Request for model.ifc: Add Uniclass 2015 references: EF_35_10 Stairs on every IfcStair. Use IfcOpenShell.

First a look at what the model holds.

```python
import ifcopenshell

model = ifcopenshell.open("model.ifc")
print(model.schema)
print("classifications:", [c.Name for c in model.by_type("IfcClassification")])
for ifc_class in ("IfcDoor", "IfcRoof", "IfcStair", "IfcWall", "IfcWindow"):
    print(ifc_class, len(model.by_type(ifc_class)))
```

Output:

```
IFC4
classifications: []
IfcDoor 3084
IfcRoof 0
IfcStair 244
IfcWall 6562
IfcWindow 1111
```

```python
import ifcopenshell
import ifcopenshell.api.classification

model = ifcopenshell.open("model.ifc")

system = ifcopenshell.api.classification.add_classification(model, classification="Uniclass 2015")

codes = {
    "IfcStair": ("EF_35_10", "Stairs"),
}
for ifc_class, (code, name) in codes.items():
    products = model.by_type(ifc_class)
    ifcopenshell.api.classification.add_reference(
        model, products=products, classification=system, identification=code, name=name
    )
    print(code, len(products))

model.write("model_updated.ifc")
```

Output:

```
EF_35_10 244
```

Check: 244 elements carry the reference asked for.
